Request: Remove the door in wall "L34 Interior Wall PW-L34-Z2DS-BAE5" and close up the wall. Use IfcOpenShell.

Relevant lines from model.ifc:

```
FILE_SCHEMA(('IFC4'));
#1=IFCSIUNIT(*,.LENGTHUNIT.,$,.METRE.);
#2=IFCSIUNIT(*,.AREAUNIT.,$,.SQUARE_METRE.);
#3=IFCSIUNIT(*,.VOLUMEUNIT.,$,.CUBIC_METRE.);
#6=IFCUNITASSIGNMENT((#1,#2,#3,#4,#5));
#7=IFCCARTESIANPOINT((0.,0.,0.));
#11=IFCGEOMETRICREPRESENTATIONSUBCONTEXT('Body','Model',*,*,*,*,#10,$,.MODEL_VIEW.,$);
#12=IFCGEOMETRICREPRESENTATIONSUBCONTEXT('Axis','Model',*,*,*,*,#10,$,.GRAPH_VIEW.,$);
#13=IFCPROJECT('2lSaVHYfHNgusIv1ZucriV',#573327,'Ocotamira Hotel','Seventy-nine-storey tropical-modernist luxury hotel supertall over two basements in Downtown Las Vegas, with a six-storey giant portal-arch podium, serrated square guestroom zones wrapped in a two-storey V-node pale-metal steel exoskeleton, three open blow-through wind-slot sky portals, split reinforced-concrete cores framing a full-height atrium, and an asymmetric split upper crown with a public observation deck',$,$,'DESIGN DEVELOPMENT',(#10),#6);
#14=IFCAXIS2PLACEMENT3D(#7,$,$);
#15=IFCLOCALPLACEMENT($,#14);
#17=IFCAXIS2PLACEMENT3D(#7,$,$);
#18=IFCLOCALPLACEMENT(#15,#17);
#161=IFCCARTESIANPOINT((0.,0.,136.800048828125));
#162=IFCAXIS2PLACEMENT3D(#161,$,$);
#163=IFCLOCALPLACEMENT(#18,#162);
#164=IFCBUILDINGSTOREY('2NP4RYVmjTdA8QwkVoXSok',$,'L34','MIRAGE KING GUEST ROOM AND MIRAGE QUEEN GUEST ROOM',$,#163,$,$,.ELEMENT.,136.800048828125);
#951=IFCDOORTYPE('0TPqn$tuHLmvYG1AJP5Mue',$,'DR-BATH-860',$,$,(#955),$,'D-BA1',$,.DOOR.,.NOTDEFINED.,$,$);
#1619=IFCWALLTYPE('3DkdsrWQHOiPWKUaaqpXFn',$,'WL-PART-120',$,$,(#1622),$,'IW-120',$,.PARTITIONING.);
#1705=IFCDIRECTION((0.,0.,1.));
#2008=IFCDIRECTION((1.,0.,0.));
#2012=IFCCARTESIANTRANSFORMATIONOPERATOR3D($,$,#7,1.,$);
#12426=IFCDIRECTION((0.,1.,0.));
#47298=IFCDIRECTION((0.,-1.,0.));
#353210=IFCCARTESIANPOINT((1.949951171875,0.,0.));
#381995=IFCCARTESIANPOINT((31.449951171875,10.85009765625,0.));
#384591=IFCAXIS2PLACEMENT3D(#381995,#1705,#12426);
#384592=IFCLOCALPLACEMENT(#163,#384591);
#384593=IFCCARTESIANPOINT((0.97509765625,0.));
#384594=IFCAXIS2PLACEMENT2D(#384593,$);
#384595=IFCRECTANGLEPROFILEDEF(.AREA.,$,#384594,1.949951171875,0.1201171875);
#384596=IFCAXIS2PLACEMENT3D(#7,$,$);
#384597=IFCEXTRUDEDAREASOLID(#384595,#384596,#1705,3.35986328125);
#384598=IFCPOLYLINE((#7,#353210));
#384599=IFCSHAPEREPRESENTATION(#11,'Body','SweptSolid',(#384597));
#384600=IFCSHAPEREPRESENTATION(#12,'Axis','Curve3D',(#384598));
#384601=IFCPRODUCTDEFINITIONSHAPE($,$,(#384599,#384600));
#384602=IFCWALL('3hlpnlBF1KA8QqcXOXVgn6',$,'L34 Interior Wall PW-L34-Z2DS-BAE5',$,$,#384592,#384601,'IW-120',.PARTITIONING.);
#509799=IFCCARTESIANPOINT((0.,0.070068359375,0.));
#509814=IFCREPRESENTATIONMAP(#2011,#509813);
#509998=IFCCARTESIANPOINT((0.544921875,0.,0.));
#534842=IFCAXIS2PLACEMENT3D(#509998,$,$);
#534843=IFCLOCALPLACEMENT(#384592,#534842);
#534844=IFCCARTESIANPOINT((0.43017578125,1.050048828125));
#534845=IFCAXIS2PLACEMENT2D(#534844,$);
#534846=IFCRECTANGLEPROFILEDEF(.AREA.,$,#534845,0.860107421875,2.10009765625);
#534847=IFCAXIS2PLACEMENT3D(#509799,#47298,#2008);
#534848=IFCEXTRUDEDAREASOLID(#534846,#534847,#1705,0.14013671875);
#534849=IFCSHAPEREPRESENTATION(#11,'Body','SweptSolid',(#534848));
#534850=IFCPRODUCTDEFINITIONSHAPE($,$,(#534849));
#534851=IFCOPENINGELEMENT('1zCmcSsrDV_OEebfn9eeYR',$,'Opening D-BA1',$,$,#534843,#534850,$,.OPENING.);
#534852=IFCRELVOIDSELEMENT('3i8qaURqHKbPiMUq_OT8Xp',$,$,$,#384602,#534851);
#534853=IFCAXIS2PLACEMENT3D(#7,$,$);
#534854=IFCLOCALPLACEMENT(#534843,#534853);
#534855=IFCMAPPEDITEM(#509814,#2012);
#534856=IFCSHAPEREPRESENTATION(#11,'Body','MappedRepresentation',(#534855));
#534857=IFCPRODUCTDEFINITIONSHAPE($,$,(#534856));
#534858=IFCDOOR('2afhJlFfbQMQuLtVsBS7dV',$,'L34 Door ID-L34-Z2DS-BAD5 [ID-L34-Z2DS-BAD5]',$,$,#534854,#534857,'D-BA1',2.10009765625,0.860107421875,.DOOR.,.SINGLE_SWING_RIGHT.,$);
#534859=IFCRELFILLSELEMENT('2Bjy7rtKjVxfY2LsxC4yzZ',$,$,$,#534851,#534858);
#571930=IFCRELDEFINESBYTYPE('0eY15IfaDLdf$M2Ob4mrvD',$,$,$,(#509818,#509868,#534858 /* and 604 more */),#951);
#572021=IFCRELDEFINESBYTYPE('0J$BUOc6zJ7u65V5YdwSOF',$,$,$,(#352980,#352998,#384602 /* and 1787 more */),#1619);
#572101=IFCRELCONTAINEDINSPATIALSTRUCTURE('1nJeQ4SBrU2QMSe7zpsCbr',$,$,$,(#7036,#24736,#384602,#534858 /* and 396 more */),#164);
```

```python
import ifcopenshell
import ifcopenshell.api.feature
import ifcopenshell.api.root
import ifcopenshell.geom
import ifcopenshell.util.shape

model = ifcopenshell.open("model.ifc")
settings = ifcopenshell.geom.settings()


def volume(element):
    """Net volume in cubic metres, openings subtracted."""
    shape = ifcopenshell.geom.create_shape(settings, element)
    return ifcopenshell.util.shape.get_volume(shape.geometry)


door = model.by_guid("2afhJlFfbQMQuLtVsBS7dV")
opening = door.FillsVoids[0].RelatingOpeningElement
wall = opening.VoidsElements[0].RelatingBuildingElement
before = volume(wall)

ifcopenshell.api.root.remove_product(model, product=door)
ifcopenshell.api.feature.remove_feature(model, feature=opening)

after = volume(wall)

print(f"wall volume {before:.3f} -> {after:.3f} m3")

model.write("model-out.ifc")
```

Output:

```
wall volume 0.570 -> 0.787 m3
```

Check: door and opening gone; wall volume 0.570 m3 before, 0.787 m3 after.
